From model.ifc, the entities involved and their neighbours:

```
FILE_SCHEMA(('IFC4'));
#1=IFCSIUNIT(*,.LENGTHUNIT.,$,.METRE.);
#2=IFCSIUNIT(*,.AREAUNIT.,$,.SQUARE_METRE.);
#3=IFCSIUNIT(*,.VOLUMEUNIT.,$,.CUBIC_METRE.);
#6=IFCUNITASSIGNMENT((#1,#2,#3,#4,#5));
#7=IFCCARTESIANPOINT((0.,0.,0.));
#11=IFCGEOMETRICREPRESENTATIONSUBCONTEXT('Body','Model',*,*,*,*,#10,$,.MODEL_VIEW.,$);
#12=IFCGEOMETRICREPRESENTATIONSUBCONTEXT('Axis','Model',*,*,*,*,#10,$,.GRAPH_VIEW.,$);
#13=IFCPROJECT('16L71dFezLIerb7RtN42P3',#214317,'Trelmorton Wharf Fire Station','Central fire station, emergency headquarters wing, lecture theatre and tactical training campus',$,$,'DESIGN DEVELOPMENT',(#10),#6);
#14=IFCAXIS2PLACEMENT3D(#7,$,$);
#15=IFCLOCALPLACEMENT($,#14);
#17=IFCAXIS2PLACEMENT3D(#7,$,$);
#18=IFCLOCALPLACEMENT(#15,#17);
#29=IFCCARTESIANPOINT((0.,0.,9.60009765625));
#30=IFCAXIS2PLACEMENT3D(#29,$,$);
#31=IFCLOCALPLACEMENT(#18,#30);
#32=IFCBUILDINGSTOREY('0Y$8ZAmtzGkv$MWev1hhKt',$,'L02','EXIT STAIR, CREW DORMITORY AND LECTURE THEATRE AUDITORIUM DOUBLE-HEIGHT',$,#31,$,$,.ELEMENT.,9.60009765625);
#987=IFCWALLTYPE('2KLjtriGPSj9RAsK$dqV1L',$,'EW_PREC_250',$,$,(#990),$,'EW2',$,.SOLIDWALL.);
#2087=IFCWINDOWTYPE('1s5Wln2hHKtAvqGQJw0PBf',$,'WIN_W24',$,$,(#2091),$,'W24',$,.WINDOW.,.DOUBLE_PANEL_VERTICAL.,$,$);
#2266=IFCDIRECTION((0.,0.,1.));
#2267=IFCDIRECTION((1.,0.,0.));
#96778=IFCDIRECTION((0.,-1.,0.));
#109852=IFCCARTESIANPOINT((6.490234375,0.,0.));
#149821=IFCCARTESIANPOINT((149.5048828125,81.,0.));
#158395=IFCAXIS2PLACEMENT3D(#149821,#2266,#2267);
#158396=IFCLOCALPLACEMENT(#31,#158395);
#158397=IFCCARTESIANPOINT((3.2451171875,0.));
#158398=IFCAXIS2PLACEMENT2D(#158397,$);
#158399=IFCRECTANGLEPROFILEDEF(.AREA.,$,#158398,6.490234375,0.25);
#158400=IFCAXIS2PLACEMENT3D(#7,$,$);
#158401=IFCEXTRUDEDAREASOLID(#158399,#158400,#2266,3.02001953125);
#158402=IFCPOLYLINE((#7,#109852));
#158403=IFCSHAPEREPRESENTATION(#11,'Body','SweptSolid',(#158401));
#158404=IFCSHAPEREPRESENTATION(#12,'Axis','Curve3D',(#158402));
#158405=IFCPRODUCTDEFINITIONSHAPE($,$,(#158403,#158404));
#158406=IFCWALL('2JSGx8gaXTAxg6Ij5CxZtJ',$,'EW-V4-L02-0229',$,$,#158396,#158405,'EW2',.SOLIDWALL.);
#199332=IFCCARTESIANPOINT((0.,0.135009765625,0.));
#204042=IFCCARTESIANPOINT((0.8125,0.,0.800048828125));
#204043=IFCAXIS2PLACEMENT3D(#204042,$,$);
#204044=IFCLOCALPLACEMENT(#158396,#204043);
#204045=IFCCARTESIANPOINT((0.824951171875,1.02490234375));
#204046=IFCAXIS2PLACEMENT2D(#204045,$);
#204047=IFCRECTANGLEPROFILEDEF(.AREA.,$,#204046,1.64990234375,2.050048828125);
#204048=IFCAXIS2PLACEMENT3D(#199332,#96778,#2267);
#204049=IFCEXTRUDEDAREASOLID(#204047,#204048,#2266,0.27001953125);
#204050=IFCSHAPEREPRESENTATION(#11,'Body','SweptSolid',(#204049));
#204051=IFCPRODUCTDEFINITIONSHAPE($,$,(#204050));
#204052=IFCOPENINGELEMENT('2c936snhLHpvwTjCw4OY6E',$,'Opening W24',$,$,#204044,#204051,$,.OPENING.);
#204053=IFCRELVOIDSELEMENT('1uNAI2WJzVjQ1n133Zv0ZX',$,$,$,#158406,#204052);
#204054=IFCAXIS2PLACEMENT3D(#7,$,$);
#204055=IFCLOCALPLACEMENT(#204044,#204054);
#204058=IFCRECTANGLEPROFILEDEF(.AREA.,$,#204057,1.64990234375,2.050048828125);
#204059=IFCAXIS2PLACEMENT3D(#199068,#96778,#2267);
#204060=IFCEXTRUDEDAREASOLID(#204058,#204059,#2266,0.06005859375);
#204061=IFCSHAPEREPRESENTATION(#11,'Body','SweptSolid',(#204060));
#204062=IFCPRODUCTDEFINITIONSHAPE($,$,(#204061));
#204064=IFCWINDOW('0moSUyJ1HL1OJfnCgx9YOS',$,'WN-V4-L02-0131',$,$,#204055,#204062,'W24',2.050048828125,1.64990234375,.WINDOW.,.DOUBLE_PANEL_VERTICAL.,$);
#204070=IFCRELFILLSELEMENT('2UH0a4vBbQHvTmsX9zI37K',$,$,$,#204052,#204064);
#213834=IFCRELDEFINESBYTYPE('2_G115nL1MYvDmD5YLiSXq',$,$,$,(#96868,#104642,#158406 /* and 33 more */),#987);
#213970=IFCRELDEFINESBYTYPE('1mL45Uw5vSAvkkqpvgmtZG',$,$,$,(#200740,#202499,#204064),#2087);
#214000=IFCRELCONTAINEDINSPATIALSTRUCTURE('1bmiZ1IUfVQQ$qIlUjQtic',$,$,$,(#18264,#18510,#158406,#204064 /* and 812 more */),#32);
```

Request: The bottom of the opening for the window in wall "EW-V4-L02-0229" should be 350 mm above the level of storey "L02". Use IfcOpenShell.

```python
import numpy as np
import ifcopenshell
import ifcopenshell.api.geometry
import ifcopenshell.geom
import ifcopenshell.util.element
import ifcopenshell.util.placement
import ifcopenshell.util.shape
import ifcopenshell.util.unit

model = ifcopenshell.open("model.ifc")
unit_scale = ifcopenshell.util.unit.calculate_unit_scale(model)

window = model.by_guid("0moSUyJ1HL1OJfnCgx9YOS")
opening = window.FillsVoids[0].RelatingOpeningElement
storey = ifcopenshell.util.element.get_container(window, ifc_class="IfcBuildingStorey")
level = ifcopenshell.util.placement.get_local_placement(storey.ObjectPlacement)[2, 3]

# The opening's origin need not be at the sill, so measure its lowest point.
shape = ifcopenshell.geom.create_shape(ifcopenshell.geom.settings(), opening)
bottom = ifcopenshell.util.shape.get_shape_bottom_elevation(shape, shape.geometry) / unit_scale
dz = level + 0.35 / unit_scale - bottom

shift = np.array([0.0, 0.0, dz])
# The window is placed relative to its opening, so it follows when the opening moves.
matrix = ifcopenshell.util.placement.get_local_placement(opening.ObjectPlacement)
matrix[:3, 3] += shift
ifcopenshell.api.geometry.edit_object_placement(
    model, product=opening, matrix=matrix, is_si=False, should_transform_children=True
)

print(f"moved by {dz * unit_scale:+.3f} m")

model.write("model-out.ifc")
```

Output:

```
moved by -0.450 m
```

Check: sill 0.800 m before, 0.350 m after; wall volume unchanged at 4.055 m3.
